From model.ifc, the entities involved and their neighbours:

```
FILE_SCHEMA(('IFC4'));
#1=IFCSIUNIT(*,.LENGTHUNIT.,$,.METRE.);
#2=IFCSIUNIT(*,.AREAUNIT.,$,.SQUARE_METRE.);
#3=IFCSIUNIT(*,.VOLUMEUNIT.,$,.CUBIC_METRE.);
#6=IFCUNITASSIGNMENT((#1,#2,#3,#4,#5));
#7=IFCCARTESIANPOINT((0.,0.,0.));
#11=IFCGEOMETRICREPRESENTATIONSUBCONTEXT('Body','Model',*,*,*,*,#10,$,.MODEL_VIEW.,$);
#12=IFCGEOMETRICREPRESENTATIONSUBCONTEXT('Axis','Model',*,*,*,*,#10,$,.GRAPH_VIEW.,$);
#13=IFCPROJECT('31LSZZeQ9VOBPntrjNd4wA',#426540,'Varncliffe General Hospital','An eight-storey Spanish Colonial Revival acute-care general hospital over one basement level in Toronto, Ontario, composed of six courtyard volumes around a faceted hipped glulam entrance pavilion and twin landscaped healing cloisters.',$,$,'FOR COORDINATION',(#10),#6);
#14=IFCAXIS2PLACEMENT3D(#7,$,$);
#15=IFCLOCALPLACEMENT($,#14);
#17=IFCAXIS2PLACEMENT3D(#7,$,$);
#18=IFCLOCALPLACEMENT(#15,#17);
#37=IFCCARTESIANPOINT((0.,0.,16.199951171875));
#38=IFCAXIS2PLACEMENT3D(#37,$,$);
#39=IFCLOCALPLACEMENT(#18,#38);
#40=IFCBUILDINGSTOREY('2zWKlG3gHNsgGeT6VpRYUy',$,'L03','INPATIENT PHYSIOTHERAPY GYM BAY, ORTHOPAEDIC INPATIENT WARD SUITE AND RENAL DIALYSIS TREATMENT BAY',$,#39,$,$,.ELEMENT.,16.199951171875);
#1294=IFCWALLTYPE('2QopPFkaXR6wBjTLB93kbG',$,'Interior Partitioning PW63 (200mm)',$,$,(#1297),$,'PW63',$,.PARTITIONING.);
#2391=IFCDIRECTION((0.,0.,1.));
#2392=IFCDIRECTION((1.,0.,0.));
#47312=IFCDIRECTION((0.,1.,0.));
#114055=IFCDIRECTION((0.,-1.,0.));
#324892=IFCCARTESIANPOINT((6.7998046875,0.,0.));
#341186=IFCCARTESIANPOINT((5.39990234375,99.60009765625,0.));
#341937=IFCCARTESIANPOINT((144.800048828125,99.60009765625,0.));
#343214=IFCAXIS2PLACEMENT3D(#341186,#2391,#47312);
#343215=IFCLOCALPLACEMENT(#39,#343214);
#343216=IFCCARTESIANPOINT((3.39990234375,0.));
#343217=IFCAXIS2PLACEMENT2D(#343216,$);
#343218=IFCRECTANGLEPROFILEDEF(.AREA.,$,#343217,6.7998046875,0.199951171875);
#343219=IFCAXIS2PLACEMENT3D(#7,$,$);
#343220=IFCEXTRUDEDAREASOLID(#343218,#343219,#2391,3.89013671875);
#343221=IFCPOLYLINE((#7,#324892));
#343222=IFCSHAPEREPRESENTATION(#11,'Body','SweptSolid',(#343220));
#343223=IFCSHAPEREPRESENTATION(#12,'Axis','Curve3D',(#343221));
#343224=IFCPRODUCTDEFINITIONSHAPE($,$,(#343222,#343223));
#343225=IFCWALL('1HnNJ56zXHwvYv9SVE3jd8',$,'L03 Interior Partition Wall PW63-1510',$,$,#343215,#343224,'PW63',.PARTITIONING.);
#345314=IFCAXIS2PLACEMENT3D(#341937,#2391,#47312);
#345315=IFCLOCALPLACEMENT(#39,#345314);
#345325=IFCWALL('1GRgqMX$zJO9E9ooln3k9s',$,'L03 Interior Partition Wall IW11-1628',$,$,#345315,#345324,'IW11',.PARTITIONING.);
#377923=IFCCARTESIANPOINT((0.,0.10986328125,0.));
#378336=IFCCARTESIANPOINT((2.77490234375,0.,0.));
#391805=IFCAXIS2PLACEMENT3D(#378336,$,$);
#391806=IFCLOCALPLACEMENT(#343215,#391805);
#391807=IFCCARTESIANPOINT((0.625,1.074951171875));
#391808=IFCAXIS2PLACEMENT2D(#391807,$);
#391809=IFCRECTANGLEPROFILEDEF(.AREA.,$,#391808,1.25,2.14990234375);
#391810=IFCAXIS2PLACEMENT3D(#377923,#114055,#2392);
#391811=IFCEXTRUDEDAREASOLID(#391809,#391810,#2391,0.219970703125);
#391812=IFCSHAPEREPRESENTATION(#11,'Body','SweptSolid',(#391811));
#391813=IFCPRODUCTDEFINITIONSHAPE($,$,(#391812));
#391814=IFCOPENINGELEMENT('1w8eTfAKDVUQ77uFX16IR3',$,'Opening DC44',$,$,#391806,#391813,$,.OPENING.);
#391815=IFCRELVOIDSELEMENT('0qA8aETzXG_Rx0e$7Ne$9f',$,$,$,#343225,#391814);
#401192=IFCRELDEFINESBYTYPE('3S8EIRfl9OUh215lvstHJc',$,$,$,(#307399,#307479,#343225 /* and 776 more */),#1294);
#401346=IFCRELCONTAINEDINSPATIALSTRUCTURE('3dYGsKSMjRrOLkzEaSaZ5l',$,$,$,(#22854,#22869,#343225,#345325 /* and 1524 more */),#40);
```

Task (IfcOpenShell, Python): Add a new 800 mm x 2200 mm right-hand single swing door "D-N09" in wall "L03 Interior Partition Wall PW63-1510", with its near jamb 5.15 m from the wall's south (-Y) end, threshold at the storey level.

```python
import numpy as np
import ifcopenshell
import ifcopenshell.api.feature
import ifcopenshell.api.geometry
import ifcopenshell.api.root
import ifcopenshell.api.spatial
import ifcopenshell.geom
import ifcopenshell.util.element
import ifcopenshell.util.placement
import ifcopenshell.util.representation
import ifcopenshell.util.shape
import ifcopenshell.util.unit

model = ifcopenshell.open("model.ifc")
unit_scale = ifcopenshell.util.unit.calculate_unit_scale(model)
settings = ifcopenshell.geom.settings()


def volume(element):
    """Net volume in cubic metres, openings subtracted."""
    shape = ifcopenshell.geom.create_shape(settings, element)
    return ifcopenshell.util.shape.get_volume(shape.geometry)


wall = model.by_id(343225)
storey = ifcopenshell.util.element.get_container(wall, ifc_class="IfcBuildingStorey")
context = ifcopenshell.util.representation.get_context(model, "Model", "Body", "MODEL_VIEW")
before = volume(wall)

width, height, from_end, sill = 0.8, 2.2, 5.15, 0.0  # metres

# The wall runs along its own X axis, and the end named is its -X end.
wall_shape = ifcopenshell.geom.create_shape(settings, wall)
x, y, z = ifcopenshell.util.shape.get_vertices(wall_shape.geometry).T
start = x.min() + from_end
face, thickness = float(y.min()), float(y.max() - y.min())
wall_matrix = ifcopenshell.util.placement.get_local_placement(wall.ObjectPlacement)
level = ifcopenshell.util.placement.get_local_placement(storey.ObjectPlacement)[2, 3]


def in_wall(x, y):
    """Placement at x, y metres in the wall's axes, at sill height."""
    matrix = wall_matrix.copy()
    matrix[:, 3] = wall_matrix @ np.array([x / unit_scale, y / unit_scale, 0.0, 1.0])
    matrix[2, 3] = level + sill / unit_scale
    return matrix


# Opening: a box that overshoots both wall faces by 50 mm.
opening = ifcopenshell.api.root.create_entity(model, ifc_class="IfcOpeningElement", predefined_type="OPENING")
box = ifcopenshell.api.geometry.add_wall_representation(
    model, context=context, length=width, height=height, thickness=thickness + 0.1
)
ifcopenshell.api.geometry.assign_representation(model, product=opening, representation=box)
ifcopenshell.api.geometry.edit_object_placement(model, product=opening, matrix=in_wall(start, face - 0.05), is_si=False)
ifcopenshell.api.feature.add_feature(model, feature=opening, element=wall)

door = ifcopenshell.api.root.create_entity(model, ifc_class="IfcDoor", name="D-N09", predefined_type="DOOR")
door.OverallWidth, door.OverallHeight = width / unit_scale, height / unit_scale
door.OperationType = "SINGLE_SWING_RIGHT"
body = ifcopenshell.api.geometry.add_door_representation(
    model,
    context=context,
    overall_width=door.OverallWidth,
    overall_height=door.OverallHeight,
    operation_type="SINGLE_SWING_RIGHT",
    lining_properties={"LiningDepth": thickness / unit_scale, "ThresholdDepth": thickness / unit_scale},
)
ifcopenshell.api.geometry.assign_representation(model, product=door, representation=body)
ifcopenshell.api.spatial.assign_container(model, products=[door], relating_structure=storey)
ifcopenshell.api.feature.add_filling(model, opening=opening, element=door)

# The lining spans the wall, so the door starts at the wall face.
ifcopenshell.api.geometry.edit_object_placement(model, product=door, matrix=in_wall(start, face), is_si=False)

after = volume(wall)

print(f"wall volume {before:.3f} -> {after:.3f} m3")

model.write("model-out.ifc")
```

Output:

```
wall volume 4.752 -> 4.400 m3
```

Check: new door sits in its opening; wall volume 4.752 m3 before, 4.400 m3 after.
